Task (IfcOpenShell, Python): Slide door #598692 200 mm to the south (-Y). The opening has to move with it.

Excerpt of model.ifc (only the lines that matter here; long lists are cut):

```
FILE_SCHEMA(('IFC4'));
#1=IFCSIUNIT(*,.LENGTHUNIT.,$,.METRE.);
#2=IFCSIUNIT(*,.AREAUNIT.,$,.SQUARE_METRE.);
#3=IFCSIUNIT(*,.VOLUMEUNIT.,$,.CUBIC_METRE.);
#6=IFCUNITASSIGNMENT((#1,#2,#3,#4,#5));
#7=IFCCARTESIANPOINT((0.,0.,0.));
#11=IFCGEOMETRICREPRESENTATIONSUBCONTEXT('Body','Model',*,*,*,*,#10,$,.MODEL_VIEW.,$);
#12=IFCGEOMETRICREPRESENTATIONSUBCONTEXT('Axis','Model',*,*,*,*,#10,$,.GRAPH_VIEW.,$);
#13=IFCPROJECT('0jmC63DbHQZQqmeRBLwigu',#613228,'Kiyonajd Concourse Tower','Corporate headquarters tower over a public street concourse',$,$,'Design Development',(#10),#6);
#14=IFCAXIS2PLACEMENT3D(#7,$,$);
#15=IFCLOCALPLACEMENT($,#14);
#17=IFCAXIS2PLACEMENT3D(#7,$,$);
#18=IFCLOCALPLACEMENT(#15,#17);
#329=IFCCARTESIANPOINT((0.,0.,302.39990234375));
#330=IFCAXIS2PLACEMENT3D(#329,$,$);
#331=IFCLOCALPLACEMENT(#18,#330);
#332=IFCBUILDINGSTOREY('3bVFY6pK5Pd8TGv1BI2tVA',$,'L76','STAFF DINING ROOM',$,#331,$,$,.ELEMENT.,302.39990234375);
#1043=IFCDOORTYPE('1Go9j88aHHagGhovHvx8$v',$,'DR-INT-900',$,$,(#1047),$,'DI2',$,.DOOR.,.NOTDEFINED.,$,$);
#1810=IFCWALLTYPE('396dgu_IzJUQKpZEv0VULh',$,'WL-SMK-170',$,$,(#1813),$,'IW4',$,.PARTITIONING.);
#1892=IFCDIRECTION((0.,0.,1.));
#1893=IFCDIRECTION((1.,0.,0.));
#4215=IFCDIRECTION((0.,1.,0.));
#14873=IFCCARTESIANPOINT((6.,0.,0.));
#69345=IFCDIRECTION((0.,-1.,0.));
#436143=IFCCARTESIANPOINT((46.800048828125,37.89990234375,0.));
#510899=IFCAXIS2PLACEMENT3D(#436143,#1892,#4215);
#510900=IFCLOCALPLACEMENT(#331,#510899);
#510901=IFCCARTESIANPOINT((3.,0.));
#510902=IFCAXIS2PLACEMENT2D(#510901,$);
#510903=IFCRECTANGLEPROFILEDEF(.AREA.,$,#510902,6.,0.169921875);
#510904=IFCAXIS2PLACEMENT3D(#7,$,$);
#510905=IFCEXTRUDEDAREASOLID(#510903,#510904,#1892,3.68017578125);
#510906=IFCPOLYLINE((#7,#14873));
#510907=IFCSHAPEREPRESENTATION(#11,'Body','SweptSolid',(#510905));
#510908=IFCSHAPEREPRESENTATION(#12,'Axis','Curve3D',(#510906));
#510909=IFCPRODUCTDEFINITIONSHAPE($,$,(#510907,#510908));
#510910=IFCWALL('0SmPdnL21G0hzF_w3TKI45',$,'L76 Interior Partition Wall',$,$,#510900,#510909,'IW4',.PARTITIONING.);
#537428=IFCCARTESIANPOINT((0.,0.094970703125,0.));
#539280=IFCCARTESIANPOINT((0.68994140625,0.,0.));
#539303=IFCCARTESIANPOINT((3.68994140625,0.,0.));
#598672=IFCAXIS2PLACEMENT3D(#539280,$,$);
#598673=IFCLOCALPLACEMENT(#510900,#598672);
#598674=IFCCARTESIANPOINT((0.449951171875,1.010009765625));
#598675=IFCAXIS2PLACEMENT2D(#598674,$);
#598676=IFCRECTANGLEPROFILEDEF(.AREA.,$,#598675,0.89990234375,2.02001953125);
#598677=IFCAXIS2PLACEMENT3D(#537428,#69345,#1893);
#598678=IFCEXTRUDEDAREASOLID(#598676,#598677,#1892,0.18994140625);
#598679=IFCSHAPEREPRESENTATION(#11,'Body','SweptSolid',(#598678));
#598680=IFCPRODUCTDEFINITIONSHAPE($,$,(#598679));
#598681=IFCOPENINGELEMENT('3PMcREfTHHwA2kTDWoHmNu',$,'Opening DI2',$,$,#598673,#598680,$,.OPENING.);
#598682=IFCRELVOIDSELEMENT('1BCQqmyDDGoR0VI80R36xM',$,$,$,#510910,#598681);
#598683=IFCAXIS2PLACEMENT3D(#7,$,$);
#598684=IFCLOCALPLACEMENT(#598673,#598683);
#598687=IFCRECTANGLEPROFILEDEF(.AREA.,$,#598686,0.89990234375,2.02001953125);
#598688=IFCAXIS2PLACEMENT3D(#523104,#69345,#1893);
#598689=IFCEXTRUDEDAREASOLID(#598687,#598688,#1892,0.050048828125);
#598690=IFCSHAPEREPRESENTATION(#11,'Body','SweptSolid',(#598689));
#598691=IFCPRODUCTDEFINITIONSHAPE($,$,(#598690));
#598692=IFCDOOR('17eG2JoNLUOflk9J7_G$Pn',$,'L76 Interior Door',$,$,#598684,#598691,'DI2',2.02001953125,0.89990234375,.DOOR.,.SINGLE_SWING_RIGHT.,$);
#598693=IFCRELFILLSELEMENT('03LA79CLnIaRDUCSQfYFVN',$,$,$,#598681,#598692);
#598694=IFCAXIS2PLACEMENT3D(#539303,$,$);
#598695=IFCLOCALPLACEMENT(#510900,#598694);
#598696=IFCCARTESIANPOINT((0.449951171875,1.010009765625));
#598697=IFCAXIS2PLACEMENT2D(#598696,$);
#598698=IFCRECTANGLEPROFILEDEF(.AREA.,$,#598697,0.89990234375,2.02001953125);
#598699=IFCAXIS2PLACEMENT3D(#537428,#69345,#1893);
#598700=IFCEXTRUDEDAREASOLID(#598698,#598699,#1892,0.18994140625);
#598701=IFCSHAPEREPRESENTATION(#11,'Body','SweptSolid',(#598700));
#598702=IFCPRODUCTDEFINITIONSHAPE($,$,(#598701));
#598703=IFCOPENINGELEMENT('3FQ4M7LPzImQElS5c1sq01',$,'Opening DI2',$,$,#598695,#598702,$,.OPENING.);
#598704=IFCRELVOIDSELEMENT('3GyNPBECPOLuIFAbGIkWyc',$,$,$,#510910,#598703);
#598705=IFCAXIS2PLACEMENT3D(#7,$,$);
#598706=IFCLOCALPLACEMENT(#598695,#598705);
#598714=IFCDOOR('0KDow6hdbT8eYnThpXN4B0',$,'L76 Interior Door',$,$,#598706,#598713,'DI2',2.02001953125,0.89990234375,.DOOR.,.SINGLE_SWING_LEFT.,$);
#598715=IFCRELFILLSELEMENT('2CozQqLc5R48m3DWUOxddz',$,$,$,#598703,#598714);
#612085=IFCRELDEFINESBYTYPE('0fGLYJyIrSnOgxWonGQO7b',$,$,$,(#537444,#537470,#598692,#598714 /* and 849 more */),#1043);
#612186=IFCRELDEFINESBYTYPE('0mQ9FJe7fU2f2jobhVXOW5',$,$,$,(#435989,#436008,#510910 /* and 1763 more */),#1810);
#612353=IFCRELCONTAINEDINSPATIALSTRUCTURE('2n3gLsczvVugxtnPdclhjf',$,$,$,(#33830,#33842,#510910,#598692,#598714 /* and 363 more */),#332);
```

```python
import ifcopenshell
import ifcopenshell.api.geometry
import ifcopenshell.util.placement
import ifcopenshell.util.unit

model = ifcopenshell.open("model.ifc")
unit_scale = ifcopenshell.util.unit.calculate_unit_scale(model)

door = model.by_guid("17eG2JoNLUOflk9J7_G$Pn")
opening = door.FillsVoids[0].RelatingOpeningElement
wall = opening.VoidsElements[0].RelatingBuildingElement

wall_matrix = ifcopenshell.util.placement.get_local_placement(wall.ObjectPlacement)
shift = wall_matrix[:3, 0] * -0.2 / unit_scale
before = ifcopenshell.util.placement.get_local_placement(door.ObjectPlacement)[:3, 3].copy()

# The door is placed relative to its opening, so it follows when the opening moves.
matrix = ifcopenshell.util.placement.get_local_placement(opening.ObjectPlacement)
matrix[:3, 3] += shift
ifcopenshell.api.geometry.edit_object_placement(
    model, product=opening, matrix=matrix, is_si=False, should_transform_children=True
)

after = ifcopenshell.util.placement.get_local_placement(door.ObjectPlacement)[:3, 3]
print("door moved by", (after - before).round(3) + 0.0)

model.write("model_updated.ifc")
```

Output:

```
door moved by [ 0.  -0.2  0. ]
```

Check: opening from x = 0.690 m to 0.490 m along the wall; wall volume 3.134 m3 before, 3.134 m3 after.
